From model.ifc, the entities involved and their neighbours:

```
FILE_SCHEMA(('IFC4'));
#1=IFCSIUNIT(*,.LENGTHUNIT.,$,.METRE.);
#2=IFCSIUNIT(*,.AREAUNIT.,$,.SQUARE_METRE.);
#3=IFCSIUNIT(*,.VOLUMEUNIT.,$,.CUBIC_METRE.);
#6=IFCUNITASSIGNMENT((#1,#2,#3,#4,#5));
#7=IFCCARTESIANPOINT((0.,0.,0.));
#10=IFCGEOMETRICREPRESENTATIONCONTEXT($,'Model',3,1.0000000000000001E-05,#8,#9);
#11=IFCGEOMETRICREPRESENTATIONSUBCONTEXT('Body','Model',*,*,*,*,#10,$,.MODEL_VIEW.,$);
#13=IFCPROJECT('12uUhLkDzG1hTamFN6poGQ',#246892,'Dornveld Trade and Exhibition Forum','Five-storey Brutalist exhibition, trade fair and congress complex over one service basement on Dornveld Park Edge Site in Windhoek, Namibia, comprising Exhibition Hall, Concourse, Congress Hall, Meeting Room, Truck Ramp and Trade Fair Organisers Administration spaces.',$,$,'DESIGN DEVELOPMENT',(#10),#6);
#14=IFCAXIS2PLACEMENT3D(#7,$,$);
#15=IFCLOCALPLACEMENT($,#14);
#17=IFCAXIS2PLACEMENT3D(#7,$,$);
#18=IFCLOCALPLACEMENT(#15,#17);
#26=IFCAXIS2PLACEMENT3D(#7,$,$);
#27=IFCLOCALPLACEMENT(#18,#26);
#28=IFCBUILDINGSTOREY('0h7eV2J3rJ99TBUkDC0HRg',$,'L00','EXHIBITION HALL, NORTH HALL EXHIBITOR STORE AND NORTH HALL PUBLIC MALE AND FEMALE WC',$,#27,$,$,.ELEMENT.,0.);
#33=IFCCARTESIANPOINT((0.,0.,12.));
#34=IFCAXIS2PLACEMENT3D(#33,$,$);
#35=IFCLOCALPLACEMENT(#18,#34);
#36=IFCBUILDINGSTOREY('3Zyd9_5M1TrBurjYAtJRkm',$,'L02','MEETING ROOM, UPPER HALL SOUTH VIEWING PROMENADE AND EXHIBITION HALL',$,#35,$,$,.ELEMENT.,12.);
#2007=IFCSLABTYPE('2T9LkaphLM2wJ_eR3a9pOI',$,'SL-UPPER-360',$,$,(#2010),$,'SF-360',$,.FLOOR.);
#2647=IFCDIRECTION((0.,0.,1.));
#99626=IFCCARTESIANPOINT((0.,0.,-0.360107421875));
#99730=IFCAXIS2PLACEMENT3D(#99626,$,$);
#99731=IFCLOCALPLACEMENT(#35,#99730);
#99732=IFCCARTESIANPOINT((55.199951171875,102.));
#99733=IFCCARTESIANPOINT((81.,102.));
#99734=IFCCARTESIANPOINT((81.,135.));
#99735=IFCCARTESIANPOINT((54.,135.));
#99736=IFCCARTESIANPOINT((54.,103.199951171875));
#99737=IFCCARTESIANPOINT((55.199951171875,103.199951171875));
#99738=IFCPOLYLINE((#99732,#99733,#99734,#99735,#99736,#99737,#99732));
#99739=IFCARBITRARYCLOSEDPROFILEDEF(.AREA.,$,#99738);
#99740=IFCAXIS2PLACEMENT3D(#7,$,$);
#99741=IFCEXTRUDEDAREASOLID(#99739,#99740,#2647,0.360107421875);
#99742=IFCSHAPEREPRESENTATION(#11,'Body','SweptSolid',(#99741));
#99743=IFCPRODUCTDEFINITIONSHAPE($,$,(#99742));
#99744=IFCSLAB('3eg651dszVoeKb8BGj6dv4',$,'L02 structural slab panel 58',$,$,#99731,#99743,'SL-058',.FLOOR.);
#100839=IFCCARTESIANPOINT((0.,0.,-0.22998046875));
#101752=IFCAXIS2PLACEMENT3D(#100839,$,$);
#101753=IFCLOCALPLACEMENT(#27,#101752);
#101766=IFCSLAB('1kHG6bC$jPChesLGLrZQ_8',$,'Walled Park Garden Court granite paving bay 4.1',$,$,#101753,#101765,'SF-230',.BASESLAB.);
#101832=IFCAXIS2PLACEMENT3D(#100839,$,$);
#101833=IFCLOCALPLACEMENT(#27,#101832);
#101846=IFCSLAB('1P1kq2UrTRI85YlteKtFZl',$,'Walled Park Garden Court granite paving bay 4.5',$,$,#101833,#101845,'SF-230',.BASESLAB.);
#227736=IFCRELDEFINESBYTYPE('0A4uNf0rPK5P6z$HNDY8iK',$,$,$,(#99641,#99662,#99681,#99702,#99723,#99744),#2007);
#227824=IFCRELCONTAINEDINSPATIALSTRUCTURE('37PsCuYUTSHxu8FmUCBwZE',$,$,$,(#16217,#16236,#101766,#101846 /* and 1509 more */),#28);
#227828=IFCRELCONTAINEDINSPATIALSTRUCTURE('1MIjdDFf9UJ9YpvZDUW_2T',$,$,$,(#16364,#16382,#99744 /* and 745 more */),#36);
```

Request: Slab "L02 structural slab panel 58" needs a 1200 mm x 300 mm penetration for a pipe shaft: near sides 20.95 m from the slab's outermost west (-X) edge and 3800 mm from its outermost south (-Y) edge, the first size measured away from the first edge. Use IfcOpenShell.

```python
import numpy as np
import ifcopenshell
import ifcopenshell.api.feature
import ifcopenshell.api.geometry
import ifcopenshell.api.root
import ifcopenshell.geom
import ifcopenshell.util.placement
import ifcopenshell.util.representation
import ifcopenshell.util.shape
import ifcopenshell.util.unit

model = ifcopenshell.open("model.ifc")
unit_scale = ifcopenshell.util.unit.calculate_unit_scale(model)
settings = ifcopenshell.geom.settings()


def volume(element):
    """Net volume in cubic metres, openings subtracted."""
    shape = ifcopenshell.geom.create_shape(settings, element)
    return ifcopenshell.util.shape.get_volume(shape.geometry)


slab = model.by_id(99744)
before = volume(slab)

# Extent in the slab's own axes, in metres. The edges named are its -X and -Y sides.
slab_shape = ifcopenshell.geom.create_shape(settings, slab)
vertices = ifcopenshell.util.shape.get_vertices(slab_shape.geometry)
x_min, y_min, bottom = vertices.min(axis=0)
top = vertices[:, 2].max()

opening = ifcopenshell.api.root.create_entity(model, ifc_class="IfcOpeningElement", name="Pipe shaft opening", predefined_type="OPENING")
context = ifcopenshell.util.representation.get_context(model, "Model", "Body", "MODEL_VIEW")
width, depth = 1.2, 0.3
outline = [(0.0, 0.0), (width, 0.0), (width, depth), (0.0, depth), (0.0, 0.0)]
# Overshoot both faces by 50 mm so the cut is clean.
shape = ifcopenshell.api.geometry.add_slab_representation(
    model, context=context, depth=top - bottom + 0.1, polyline=outline
)
ifcopenshell.api.geometry.assign_representation(model, product=opening, representation=shape)

matrix = ifcopenshell.util.placement.get_local_placement(slab.ObjectPlacement)
matrix[:, 3] = matrix @ np.append(np.array([x_min + 20.95, y_min + 3.8, bottom - 0.05]) / unit_scale, 1.0)
ifcopenshell.api.geometry.edit_object_placement(model, product=opening, matrix=matrix, is_si=False)
ifcopenshell.api.feature.add_feature(model, feature=opening, element=slab)

after = volume(slab)

print(f"slab volume {before:.3f} -> {after:.3f} m3")

model.write("model-out.ifc")
```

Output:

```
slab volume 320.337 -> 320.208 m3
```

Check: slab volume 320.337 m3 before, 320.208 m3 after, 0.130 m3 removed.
